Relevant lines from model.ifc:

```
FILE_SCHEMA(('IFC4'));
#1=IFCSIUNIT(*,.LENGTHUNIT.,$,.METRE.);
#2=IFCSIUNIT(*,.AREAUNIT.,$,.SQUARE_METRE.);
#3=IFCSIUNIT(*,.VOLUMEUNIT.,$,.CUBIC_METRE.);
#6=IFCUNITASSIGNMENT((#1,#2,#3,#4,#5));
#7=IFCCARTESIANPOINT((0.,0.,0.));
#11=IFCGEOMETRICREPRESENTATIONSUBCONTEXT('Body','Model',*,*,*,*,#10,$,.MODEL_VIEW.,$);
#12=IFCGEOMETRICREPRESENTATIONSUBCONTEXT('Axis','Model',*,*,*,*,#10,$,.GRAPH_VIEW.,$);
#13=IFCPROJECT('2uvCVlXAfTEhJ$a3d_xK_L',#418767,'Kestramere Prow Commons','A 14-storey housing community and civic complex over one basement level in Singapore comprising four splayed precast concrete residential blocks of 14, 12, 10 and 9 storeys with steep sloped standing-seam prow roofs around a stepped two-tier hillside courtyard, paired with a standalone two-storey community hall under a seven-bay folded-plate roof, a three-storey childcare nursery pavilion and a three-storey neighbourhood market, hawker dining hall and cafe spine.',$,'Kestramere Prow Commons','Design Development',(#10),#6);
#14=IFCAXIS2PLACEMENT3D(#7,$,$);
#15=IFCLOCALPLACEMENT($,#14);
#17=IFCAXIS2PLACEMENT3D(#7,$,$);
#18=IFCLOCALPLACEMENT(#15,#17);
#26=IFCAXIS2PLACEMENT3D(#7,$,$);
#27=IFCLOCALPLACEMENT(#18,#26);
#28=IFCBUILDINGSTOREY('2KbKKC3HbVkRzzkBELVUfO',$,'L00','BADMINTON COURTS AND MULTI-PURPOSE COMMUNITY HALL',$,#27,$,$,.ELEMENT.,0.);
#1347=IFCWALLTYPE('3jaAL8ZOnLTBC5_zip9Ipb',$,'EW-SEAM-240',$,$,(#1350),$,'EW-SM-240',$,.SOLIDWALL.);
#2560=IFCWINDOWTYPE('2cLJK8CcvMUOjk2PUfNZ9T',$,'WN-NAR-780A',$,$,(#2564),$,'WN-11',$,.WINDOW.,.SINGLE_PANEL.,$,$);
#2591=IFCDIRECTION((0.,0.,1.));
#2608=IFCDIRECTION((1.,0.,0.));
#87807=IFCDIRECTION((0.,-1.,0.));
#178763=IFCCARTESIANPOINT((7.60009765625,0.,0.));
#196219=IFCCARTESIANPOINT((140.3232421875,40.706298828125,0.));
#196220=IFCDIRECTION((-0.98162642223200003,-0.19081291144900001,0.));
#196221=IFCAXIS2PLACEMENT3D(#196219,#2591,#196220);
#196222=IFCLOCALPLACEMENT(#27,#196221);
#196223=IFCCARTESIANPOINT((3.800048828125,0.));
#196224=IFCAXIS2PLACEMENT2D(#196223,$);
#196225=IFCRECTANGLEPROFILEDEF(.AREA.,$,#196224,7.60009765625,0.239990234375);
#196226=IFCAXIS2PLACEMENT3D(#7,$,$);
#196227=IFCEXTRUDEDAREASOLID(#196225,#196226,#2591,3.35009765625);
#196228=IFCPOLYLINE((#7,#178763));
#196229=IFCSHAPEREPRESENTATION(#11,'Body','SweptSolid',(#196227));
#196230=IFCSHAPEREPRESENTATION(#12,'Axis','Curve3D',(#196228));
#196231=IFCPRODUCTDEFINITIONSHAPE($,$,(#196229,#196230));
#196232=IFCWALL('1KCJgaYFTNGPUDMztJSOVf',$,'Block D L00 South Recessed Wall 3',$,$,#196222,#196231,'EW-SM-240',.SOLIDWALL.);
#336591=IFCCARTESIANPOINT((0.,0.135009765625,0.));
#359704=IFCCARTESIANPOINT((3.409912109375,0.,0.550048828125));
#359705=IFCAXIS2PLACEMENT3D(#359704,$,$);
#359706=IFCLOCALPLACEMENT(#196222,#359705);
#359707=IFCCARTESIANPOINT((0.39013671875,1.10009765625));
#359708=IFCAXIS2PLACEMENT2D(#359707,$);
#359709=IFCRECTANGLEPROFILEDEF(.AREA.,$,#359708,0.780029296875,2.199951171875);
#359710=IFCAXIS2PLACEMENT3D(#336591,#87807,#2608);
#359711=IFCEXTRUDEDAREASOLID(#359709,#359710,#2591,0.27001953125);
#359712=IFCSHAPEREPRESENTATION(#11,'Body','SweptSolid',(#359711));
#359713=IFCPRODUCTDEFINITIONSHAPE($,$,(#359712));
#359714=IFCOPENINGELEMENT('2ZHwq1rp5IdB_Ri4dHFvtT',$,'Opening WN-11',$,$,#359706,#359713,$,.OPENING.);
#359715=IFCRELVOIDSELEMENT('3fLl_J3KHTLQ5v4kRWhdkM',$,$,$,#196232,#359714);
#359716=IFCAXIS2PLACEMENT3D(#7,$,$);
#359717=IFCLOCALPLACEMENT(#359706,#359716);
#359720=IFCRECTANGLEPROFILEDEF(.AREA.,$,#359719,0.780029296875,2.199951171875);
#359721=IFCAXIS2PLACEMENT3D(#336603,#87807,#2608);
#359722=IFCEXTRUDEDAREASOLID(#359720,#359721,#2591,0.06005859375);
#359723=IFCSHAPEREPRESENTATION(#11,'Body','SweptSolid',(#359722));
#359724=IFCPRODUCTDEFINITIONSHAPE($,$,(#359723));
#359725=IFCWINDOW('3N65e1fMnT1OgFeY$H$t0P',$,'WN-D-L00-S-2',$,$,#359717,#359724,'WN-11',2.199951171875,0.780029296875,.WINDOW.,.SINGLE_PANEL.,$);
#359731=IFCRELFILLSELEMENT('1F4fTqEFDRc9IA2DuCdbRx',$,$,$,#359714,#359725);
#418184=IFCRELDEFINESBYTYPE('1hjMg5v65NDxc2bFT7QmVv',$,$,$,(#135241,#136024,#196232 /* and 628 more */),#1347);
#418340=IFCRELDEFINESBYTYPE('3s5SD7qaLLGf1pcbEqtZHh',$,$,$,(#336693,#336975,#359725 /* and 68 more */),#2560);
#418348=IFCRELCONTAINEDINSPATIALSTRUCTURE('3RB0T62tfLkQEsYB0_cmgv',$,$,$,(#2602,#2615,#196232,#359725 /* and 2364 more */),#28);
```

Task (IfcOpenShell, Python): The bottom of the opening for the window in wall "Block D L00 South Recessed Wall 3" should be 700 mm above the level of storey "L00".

```python
import numpy as np
import ifcopenshell
import ifcopenshell.api.geometry
import ifcopenshell.geom
import ifcopenshell.util.element
import ifcopenshell.util.placement
import ifcopenshell.util.shape
import ifcopenshell.util.unit

model = ifcopenshell.open("model.ifc")
unit_scale = ifcopenshell.util.unit.calculate_unit_scale(model)

window = model.by_guid("3N65e1fMnT1OgFeY$H$t0P")
opening = window.FillsVoids[0].RelatingOpeningElement
storey = ifcopenshell.util.element.get_container(window, ifc_class="IfcBuildingStorey")
level = ifcopenshell.util.placement.get_local_placement(storey.ObjectPlacement)[2, 3]

# The opening's origin need not be at the sill, so measure its lowest point.
shape = ifcopenshell.geom.create_shape(ifcopenshell.geom.settings(), opening)
bottom = ifcopenshell.util.shape.get_shape_bottom_elevation(shape, shape.geometry) / unit_scale
dz = level + 0.7 - bottom

shift = np.array([0.0, 0.0, dz])
# The window is placed relative to its opening, so it follows when the opening moves.
matrix = ifcopenshell.util.placement.get_local_placement(opening.ObjectPlacement)
matrix[:3, 3] += shift
ifcopenshell.api.geometry.edit_object_placement(
    model, product=opening, matrix=matrix, is_si=False, should_transform_children=True
)

print(f"moved by {dz * unit_scale:+.3f} m")

model.write("model_edited.ifc")
```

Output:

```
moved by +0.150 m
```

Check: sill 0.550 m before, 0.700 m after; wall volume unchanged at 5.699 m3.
